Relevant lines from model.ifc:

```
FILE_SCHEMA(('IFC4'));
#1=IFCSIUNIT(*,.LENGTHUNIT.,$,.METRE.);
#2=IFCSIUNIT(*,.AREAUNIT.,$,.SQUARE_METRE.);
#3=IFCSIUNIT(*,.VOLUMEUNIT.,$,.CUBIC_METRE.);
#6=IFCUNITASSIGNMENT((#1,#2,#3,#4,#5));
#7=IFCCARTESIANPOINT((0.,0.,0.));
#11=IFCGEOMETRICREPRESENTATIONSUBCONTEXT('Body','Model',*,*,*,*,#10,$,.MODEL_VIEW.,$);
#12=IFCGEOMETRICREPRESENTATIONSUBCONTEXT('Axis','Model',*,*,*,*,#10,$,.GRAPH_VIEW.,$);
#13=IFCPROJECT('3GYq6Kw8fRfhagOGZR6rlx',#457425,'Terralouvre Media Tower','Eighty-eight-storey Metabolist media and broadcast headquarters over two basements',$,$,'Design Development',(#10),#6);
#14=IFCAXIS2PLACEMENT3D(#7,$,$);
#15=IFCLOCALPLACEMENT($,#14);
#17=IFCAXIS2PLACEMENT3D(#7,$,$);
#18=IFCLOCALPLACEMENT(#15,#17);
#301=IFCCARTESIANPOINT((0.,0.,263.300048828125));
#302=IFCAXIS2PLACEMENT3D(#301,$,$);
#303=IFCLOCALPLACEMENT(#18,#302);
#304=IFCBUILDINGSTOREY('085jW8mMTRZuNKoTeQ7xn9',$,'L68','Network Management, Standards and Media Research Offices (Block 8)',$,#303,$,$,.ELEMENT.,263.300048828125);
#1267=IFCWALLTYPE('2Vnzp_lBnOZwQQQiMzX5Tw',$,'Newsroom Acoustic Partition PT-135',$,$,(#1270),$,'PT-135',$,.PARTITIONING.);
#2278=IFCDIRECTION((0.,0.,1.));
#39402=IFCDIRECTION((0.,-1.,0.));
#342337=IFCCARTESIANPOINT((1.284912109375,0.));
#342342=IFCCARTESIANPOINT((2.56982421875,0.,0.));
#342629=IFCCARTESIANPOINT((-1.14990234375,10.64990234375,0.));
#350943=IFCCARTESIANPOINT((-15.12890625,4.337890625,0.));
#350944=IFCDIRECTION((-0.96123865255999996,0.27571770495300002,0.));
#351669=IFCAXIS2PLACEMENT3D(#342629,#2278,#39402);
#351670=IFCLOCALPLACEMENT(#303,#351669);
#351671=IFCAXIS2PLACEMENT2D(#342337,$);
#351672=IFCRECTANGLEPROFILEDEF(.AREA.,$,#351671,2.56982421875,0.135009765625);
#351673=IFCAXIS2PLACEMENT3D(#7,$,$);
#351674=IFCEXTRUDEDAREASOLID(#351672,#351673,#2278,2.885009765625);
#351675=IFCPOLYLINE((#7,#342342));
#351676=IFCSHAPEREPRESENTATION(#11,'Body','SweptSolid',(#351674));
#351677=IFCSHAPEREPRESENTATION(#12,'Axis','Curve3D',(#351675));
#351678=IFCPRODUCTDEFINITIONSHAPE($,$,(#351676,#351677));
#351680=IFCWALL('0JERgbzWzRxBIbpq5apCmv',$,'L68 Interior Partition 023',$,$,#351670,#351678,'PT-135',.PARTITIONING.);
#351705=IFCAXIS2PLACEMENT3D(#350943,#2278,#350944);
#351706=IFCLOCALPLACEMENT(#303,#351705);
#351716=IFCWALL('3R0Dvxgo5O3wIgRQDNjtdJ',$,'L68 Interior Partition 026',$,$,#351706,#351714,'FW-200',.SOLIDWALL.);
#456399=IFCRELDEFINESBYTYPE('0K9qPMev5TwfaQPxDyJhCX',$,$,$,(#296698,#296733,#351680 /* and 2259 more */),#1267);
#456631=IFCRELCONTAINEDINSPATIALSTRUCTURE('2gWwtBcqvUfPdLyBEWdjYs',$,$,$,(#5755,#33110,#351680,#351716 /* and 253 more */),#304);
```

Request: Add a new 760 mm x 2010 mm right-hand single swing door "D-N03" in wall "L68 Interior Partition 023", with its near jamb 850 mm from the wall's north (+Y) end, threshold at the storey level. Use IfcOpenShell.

```python
import numpy as np
import ifcopenshell
import ifcopenshell.api.feature
import ifcopenshell.api.geometry
import ifcopenshell.api.root
import ifcopenshell.api.spatial
import ifcopenshell.geom
import ifcopenshell.util.element
import ifcopenshell.util.placement
import ifcopenshell.util.representation
import ifcopenshell.util.shape
import ifcopenshell.util.unit

model = ifcopenshell.open("model.ifc")
unit_scale = ifcopenshell.util.unit.calculate_unit_scale(model)
settings = ifcopenshell.geom.settings()


def volume(element):
    """Net volume in cubic metres, openings subtracted."""
    shape = ifcopenshell.geom.create_shape(settings, element)
    return ifcopenshell.util.shape.get_volume(shape.geometry)


wall = model.by_id(351680)
storey = ifcopenshell.util.element.get_container(wall, ifc_class="IfcBuildingStorey")
context = ifcopenshell.util.representation.get_context(model, "Model", "Body", "MODEL_VIEW")
before = volume(wall)

width, height, from_end, sill = 0.76, 2.01, 0.85, 0.0  # metres

# The wall runs along its own X axis, and the end named is its -X end.
wall_shape = ifcopenshell.geom.create_shape(settings, wall)
x, y, z = ifcopenshell.util.shape.get_vertices(wall_shape.geometry).T
start = x.min() + from_end
face, thickness = float(y.min()), float(y.max() - y.min())
wall_matrix = ifcopenshell.util.placement.get_local_placement(wall.ObjectPlacement)
level = ifcopenshell.util.placement.get_local_placement(storey.ObjectPlacement)[2, 3]


def in_wall(x, y):
    """Placement at x, y metres in the wall's axes, at sill height."""
    matrix = wall_matrix.copy()
    matrix[:, 3] = wall_matrix @ np.array([x / unit_scale, y / unit_scale, 0.0, 1.0])
    matrix[2, 3] = level + sill / unit_scale
    return matrix


# Opening: a box that overshoots both wall faces by 50 mm.
opening = ifcopenshell.api.root.create_entity(model, ifc_class="IfcOpeningElement", predefined_type="OPENING")
box = ifcopenshell.api.geometry.add_wall_representation(
    model, context=context, length=width, height=height, thickness=thickness + 0.1
)
ifcopenshell.api.geometry.assign_representation(model, product=opening, representation=box)
ifcopenshell.api.geometry.edit_object_placement(model, product=opening, matrix=in_wall(start, face - 0.05), is_si=False)
ifcopenshell.api.feature.add_feature(model, feature=opening, element=wall)

door = ifcopenshell.api.root.create_entity(model, ifc_class="IfcDoor", name="D-N03", predefined_type="DOOR")
door.OverallWidth, door.OverallHeight = width / unit_scale, height / unit_scale
door.OperationType = "SINGLE_SWING_RIGHT"
body = ifcopenshell.api.geometry.add_door_representation(
    model,
    context=context,
    overall_width=door.OverallWidth,
    overall_height=door.OverallHeight,
    operation_type="SINGLE_SWING_RIGHT",
    lining_properties={"LiningDepth": thickness / unit_scale, "ThresholdDepth": thickness / unit_scale},
)
ifcopenshell.api.geometry.assign_representation(model, product=door, representation=body)
ifcopenshell.api.spatial.assign_container(model, products=[door], relating_structure=storey)
ifcopenshell.api.feature.add_filling(model, opening=opening, element=door)

# The lining spans the wall, so the door starts at the wall face.
ifcopenshell.api.geometry.edit_object_placement(model, product=door, matrix=in_wall(start, face), is_si=False)

after = volume(wall)

print(f"wall volume {before:.3f} -> {after:.3f} m3")

model.write("model_rev.ifc")
```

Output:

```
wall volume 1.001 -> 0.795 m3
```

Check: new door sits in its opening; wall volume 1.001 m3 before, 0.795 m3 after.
